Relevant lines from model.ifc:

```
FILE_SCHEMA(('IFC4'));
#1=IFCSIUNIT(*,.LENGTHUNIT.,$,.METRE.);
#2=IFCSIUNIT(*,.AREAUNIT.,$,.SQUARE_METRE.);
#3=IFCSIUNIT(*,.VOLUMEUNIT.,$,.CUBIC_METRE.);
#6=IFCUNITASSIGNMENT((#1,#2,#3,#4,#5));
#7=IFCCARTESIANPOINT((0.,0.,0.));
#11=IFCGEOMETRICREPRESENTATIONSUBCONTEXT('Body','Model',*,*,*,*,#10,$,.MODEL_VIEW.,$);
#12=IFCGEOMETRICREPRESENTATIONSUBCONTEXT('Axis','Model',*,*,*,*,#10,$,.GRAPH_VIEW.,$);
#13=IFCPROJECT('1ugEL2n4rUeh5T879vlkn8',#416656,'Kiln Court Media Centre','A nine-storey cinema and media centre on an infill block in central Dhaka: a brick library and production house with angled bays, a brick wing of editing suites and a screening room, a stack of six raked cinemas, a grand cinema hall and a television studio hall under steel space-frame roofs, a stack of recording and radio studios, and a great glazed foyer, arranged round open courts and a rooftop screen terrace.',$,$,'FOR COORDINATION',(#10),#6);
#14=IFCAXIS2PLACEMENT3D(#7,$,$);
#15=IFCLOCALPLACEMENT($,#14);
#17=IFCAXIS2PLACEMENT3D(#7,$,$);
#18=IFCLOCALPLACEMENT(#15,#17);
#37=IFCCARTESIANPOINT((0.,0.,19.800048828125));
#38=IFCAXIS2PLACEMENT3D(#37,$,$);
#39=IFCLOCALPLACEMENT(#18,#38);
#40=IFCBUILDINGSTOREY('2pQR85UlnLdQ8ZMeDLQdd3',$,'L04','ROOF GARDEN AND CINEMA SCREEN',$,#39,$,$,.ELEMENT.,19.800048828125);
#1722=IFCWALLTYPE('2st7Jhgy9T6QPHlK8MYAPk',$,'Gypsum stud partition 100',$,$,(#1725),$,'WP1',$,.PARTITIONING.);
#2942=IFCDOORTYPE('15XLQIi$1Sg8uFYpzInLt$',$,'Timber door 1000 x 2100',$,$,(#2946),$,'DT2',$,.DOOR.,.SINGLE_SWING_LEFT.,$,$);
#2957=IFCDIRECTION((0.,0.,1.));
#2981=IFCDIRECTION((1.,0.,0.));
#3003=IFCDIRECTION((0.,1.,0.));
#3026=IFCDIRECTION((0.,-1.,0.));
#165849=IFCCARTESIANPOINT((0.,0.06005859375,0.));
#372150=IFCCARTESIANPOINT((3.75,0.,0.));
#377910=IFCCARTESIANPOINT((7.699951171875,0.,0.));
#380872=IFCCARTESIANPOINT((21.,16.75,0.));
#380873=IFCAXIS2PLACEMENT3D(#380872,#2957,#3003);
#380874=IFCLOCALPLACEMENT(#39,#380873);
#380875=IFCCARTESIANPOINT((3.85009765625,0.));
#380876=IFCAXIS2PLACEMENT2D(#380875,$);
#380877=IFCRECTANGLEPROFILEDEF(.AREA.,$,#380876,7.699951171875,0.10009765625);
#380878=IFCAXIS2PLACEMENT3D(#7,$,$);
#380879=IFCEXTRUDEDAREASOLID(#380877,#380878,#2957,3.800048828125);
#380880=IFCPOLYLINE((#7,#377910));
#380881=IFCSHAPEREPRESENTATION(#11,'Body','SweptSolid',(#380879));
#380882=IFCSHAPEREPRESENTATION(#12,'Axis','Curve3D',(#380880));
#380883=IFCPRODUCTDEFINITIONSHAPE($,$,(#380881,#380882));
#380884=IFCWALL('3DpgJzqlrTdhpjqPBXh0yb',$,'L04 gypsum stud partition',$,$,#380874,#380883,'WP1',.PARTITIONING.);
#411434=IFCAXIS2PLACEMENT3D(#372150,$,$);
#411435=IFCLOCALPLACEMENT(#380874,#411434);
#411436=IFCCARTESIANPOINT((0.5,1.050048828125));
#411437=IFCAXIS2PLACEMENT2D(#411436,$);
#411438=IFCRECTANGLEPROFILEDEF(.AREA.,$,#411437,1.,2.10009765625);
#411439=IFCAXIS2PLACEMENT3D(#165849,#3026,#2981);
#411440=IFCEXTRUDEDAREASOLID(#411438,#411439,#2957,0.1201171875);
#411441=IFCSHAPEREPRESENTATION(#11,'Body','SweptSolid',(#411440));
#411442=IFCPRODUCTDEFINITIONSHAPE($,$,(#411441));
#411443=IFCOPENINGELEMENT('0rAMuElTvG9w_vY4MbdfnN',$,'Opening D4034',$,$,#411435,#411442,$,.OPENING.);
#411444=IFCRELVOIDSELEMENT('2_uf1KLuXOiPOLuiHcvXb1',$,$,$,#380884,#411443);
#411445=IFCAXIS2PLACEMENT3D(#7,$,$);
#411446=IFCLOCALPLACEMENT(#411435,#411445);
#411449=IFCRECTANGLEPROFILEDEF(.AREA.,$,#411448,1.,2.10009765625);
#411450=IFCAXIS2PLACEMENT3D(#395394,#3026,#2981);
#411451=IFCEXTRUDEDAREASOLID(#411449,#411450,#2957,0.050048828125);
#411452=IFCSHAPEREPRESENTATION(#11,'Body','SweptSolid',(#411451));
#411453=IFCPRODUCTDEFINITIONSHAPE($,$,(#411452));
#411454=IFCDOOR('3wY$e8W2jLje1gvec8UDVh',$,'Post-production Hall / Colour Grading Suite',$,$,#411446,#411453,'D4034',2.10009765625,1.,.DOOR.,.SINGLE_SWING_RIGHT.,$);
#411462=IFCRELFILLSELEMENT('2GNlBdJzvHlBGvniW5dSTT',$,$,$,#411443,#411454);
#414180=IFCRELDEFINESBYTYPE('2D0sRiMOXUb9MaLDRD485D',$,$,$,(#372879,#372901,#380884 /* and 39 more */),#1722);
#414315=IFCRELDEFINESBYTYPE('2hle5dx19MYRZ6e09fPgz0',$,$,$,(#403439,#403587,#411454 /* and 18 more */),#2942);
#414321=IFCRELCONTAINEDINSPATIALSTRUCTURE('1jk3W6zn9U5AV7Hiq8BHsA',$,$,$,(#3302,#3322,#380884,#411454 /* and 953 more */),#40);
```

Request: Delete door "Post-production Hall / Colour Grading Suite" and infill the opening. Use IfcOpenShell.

```python
import ifcopenshell
import ifcopenshell.api.feature
import ifcopenshell.api.root
import ifcopenshell.geom
import ifcopenshell.util.shape

model = ifcopenshell.open("model.ifc")
settings = ifcopenshell.geom.settings()


def volume(element):
    """Net volume in cubic metres, openings subtracted."""
    shape = ifcopenshell.geom.create_shape(settings, element)
    return ifcopenshell.util.shape.get_volume(shape.geometry)


door = model.by_guid("3wY$e8W2jLje1gvec8UDVh")
opening = door.FillsVoids[0].RelatingOpeningElement
wall = opening.VoidsElements[0].RelatingBuildingElement
before = volume(wall)

ifcopenshell.api.root.remove_product(model, product=door)
ifcopenshell.api.feature.remove_feature(model, feature=opening)

after = volume(wall)

print(f"wall volume {before:.3f} -> {after:.3f} m3")

model.write("model_rev.ifc")
```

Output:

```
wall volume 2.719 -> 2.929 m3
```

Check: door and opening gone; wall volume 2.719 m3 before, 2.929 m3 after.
